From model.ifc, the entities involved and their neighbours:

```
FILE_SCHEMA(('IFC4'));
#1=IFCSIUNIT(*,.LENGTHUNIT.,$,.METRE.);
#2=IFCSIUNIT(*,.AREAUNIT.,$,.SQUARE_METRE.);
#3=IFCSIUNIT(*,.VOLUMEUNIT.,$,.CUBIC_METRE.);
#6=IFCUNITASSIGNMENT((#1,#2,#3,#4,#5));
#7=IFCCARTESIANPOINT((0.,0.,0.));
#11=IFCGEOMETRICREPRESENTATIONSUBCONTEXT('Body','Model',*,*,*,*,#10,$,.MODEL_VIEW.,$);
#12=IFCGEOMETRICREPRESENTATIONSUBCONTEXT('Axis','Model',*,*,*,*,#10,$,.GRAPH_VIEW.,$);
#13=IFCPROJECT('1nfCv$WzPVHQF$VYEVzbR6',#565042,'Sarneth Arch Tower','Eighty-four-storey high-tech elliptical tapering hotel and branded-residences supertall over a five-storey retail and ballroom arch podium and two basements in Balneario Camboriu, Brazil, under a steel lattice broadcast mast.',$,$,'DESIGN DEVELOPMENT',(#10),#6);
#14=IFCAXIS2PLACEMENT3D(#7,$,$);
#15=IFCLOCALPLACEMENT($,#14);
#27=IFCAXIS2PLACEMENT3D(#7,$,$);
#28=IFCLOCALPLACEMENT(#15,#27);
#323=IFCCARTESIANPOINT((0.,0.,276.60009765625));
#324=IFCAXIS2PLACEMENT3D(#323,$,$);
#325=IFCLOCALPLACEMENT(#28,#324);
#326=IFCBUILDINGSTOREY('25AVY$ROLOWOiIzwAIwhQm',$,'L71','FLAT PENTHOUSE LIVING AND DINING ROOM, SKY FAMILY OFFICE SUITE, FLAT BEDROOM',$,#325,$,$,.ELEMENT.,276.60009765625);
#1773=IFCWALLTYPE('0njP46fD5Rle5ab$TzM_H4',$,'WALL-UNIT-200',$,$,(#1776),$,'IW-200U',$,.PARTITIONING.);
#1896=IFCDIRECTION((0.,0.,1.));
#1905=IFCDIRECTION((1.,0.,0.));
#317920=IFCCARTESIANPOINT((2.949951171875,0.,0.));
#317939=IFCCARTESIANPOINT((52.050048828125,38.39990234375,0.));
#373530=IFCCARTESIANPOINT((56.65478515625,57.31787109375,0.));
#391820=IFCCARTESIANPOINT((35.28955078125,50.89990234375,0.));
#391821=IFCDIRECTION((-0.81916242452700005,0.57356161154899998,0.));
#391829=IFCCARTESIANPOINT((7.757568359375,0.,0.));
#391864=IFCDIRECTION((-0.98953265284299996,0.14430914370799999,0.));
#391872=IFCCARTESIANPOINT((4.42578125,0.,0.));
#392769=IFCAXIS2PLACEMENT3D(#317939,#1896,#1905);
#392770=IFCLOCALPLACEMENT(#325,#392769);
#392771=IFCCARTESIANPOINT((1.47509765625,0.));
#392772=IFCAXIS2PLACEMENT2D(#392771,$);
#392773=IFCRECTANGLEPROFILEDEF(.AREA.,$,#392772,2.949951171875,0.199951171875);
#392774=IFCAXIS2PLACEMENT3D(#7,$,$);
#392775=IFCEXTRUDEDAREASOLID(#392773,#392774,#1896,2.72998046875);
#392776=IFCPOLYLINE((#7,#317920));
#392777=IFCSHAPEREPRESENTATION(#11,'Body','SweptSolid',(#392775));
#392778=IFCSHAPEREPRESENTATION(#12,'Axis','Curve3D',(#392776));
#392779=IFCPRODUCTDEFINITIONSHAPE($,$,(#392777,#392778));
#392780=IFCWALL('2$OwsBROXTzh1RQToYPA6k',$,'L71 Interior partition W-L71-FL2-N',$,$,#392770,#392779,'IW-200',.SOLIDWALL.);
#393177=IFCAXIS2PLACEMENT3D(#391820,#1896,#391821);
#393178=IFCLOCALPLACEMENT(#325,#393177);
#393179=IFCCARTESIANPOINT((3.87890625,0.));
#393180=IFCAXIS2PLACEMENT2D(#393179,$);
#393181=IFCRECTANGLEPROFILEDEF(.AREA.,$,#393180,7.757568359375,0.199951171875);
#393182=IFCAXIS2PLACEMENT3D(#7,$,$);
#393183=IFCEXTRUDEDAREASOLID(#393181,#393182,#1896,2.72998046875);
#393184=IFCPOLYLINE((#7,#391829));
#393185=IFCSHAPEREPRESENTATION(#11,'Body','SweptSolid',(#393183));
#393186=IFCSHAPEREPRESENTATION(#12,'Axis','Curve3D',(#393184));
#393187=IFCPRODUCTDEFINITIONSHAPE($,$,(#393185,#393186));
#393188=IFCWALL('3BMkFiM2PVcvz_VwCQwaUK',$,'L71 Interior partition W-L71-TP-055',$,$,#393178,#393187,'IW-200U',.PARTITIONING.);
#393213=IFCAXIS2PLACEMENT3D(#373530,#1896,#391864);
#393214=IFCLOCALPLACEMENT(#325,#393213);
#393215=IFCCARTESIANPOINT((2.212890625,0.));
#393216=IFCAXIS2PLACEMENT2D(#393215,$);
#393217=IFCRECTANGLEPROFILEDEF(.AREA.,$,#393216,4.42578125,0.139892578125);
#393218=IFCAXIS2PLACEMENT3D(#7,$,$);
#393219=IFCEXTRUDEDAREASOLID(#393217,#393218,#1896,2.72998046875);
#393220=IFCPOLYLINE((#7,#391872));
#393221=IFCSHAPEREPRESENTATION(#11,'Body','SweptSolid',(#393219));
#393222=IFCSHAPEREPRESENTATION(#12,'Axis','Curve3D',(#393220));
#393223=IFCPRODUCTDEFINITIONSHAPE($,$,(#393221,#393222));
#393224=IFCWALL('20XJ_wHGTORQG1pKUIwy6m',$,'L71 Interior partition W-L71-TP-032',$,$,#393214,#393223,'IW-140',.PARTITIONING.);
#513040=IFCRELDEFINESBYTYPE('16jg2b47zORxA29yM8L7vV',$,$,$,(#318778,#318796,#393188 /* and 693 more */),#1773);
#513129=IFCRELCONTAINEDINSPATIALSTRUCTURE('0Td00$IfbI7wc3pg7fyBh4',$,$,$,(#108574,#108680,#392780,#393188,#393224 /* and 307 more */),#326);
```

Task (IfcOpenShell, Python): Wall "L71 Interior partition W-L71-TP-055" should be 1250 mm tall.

```python
import ifcopenshell
import ifcopenshell.geom
import ifcopenshell.util.representation
import ifcopenshell.util.shape
import ifcopenshell.util.unit

model = ifcopenshell.open("model.ifc")
unit_scale = ifcopenshell.util.unit.calculate_unit_scale(model)
settings = ifcopenshell.geom.settings()


def volume(element):
    """Net volume in cubic metres, openings subtracted."""
    shape = ifcopenshell.geom.create_shape(settings, element)
    return ifcopenshell.util.shape.get_volume(shape.geometry)


wall = model.by_guid("3BMkFiM2PVcvz_VwCQwaUK")
before = volume(wall)

body = ifcopenshell.util.representation.get_representation(wall, "Model", "Body")
solid = body.Items[0]
old_height = solid.Depth
solid.Depth = 1.25 / unit_scale
after = volume(wall)

print(f"height {old_height:g} -> {solid.Depth:g}, volume {before:.3f} -> {after:.3f} m3")

model.write("model_updated.ifc")
```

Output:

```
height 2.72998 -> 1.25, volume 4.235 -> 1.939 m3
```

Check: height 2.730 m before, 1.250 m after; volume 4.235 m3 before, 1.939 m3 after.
